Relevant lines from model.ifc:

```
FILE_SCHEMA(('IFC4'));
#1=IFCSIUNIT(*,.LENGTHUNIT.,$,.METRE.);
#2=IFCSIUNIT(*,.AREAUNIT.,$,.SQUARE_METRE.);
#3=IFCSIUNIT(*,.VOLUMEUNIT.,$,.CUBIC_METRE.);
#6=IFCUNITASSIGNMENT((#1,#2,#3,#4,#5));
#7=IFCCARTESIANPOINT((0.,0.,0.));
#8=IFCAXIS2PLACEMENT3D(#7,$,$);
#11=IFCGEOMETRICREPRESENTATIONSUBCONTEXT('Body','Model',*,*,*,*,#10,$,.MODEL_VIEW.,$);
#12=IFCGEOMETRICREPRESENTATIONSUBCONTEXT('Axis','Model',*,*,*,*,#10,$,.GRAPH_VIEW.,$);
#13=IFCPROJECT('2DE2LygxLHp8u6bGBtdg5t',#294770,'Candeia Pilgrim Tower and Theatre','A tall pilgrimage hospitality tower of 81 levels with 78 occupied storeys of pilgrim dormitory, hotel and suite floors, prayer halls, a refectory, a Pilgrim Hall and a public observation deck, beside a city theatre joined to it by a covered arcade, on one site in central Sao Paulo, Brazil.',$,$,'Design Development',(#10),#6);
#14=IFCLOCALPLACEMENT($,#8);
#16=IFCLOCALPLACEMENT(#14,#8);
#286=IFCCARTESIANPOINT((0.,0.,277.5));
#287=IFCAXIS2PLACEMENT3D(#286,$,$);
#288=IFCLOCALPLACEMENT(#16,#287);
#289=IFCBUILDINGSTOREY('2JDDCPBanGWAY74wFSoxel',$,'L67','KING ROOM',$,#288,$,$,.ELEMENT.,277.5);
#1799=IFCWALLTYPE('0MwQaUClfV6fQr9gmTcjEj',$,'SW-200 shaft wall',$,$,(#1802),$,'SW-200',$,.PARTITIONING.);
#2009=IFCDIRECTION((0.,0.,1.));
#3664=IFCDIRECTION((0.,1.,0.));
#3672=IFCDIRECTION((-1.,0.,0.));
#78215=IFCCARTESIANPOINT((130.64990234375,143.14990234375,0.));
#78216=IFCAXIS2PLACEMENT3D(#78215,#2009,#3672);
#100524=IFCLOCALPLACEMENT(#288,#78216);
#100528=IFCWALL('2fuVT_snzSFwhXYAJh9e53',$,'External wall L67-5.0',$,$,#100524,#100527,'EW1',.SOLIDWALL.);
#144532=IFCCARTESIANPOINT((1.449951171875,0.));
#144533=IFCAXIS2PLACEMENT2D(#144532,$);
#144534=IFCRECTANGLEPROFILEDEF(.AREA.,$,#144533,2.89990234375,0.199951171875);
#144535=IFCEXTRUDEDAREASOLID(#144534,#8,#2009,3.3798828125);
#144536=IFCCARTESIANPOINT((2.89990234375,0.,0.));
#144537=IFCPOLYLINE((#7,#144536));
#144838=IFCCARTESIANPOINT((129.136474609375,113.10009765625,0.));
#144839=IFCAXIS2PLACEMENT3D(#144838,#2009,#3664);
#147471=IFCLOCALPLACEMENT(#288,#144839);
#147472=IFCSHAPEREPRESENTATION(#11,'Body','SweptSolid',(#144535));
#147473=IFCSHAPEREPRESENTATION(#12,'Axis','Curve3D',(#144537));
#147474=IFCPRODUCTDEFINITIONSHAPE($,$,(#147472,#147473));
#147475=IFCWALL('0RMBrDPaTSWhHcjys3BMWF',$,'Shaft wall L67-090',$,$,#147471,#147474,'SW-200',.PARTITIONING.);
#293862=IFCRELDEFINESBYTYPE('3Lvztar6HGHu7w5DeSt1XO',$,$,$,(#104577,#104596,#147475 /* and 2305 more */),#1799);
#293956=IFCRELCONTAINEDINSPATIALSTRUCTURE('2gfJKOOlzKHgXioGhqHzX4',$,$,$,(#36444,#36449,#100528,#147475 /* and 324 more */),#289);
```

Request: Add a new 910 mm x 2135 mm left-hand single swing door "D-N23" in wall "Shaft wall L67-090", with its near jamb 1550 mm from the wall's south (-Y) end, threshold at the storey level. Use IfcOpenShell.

```python
import numpy as np
import ifcopenshell
import ifcopenshell.api.feature
import ifcopenshell.api.geometry
import ifcopenshell.api.root
import ifcopenshell.api.spatial
import ifcopenshell.geom
import ifcopenshell.util.element
import ifcopenshell.util.placement
import ifcopenshell.util.representation
import ifcopenshell.util.shape
import ifcopenshell.util.unit

model = ifcopenshell.open("model.ifc")
unit_scale = ifcopenshell.util.unit.calculate_unit_scale(model)
settings = ifcopenshell.geom.settings()


def volume(element):
    """Net volume in cubic metres, openings subtracted."""
    shape = ifcopenshell.geom.create_shape(settings, element)
    return ifcopenshell.util.shape.get_volume(shape.geometry)


wall = model.by_id(147475)
storey = ifcopenshell.util.element.get_container(wall, ifc_class="IfcBuildingStorey")
context = ifcopenshell.util.representation.get_context(model, "Model", "Body", "MODEL_VIEW")
before = volume(wall)

width, height, from_end, sill = 0.91, 2.135, 1.55, 0.0  # metres

# The wall runs along its own X axis, and the end named is its -X end.
wall_shape = ifcopenshell.geom.create_shape(settings, wall)
x, y, z = ifcopenshell.util.shape.get_vertices(wall_shape.geometry).T
start = x.min() + from_end
face, thickness = float(y.min()), float(y.max() - y.min())
wall_matrix = ifcopenshell.util.placement.get_local_placement(wall.ObjectPlacement)
level = ifcopenshell.util.placement.get_local_placement(storey.ObjectPlacement)[2, 3]


def in_wall(x, y):
    """Placement at x, y metres in the wall's axes, at sill height."""
    matrix = wall_matrix.copy()
    matrix[:, 3] = wall_matrix @ np.array([x / unit_scale, y / unit_scale, 0.0, 1.0])
    matrix[2, 3] = level + sill / unit_scale
    return matrix


# Opening: a box that overshoots both wall faces by 50 mm.
opening = ifcopenshell.api.root.create_entity(model, ifc_class="IfcOpeningElement", predefined_type="OPENING")
box = ifcopenshell.api.geometry.add_wall_representation(
    model, context=context, length=width, height=height, thickness=thickness + 0.1
)
ifcopenshell.api.geometry.assign_representation(model, product=opening, representation=box)
ifcopenshell.api.geometry.edit_object_placement(model, product=opening, matrix=in_wall(start, face - 0.05), is_si=False)
ifcopenshell.api.feature.add_feature(model, feature=opening, element=wall)

door = ifcopenshell.api.root.create_entity(model, ifc_class="IfcDoor", name="D-N23", predefined_type="DOOR")
door.OverallWidth, door.OverallHeight = width / unit_scale, height / unit_scale
door.OperationType = "SINGLE_SWING_LEFT"
body = ifcopenshell.api.geometry.add_door_representation(
    model,
    context=context,
    overall_width=door.OverallWidth,
    overall_height=door.OverallHeight,
    operation_type="SINGLE_SWING_LEFT",
    lining_properties={"LiningDepth": thickness / unit_scale, "ThresholdDepth": thickness / unit_scale},
)
ifcopenshell.api.geometry.assign_representation(model, product=door, representation=body)
ifcopenshell.api.spatial.assign_container(model, products=[door], relating_structure=storey)
ifcopenshell.api.feature.add_filling(model, opening=opening, element=door)

# The lining spans the wall, so the door starts at the wall face.
ifcopenshell.api.geometry.edit_object_placement(model, product=door, matrix=in_wall(start, face), is_si=False)

after = volume(wall)

print(f"wall volume {before:.3f} -> {after:.3f} m3")

model.write("model-out.ifc")
```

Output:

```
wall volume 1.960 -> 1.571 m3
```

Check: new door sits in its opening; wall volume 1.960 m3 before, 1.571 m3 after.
